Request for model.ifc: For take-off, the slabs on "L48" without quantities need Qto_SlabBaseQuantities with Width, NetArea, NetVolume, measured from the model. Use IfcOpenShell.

First a look at what the model holds.

```python
import ifcopenshell
import ifcopenshell.util.element
import ifcopenshell.util.unit

model = ifcopenshell.open("model.ifc")
print(model.schema)
for unit_type in ("LENGTHUNIT", "AREAUNIT", "VOLUMEUNIT"):
    print(unit_type, ifcopenshell.util.unit.calculate_unit_scale(model, unit_type))
storey = next(s for s in model.by_type("IfcBuildingStorey") if s.Name == "L48")
slabs = [e for e in ifcopenshell.util.element.get_decomposition(storey) if e.is_a("IfcSlab")]
for e in sorted(slabs, key=lambda e: e.id()):
    print(e.id(), e.is_a(), e.Name, list(ifcopenshell.util.element.get_psets(e, qtos_only=True)), sep=" | ")
```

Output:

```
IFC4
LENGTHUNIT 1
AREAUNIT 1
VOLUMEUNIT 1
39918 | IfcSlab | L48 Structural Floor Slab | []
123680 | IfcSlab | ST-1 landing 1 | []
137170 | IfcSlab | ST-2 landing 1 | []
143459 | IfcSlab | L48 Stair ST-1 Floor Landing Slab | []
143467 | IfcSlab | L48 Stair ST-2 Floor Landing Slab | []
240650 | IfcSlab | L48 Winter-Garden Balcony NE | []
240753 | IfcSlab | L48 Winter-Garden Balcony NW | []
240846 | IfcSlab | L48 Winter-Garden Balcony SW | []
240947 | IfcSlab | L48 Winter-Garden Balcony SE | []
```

```python
import ifcopenshell
import ifcopenshell.api.pset
import ifcopenshell.geom
import ifcopenshell.util.element
import ifcopenshell.util.shape
import ifcopenshell.util.unit

model = ifcopenshell.open("model.ifc")
unit_scale = ifcopenshell.util.unit.calculate_unit_scale(model)
area_scale = ifcopenshell.util.unit.calculate_unit_scale(model, "AREAUNIT")
volume_scale = ifcopenshell.util.unit.calculate_unit_scale(model, "VOLUMEUNIT")
settings = ifcopenshell.geom.settings()

storey = next(s for s in model.by_type("IfcBuildingStorey") if s.Name == "L48")
slabs = [e for e in ifcopenshell.util.element.get_decomposition(storey) if e.is_a("IfcSlab")]

for e in sorted(slabs, key=lambda e: e.id()):
    if ifcopenshell.util.element.get_psets(e, qtos_only=True, should_inherit=False):
        continue
    # Geometry comes back in metres, in the element's own axes.
    shape = ifcopenshell.geom.create_shape(settings, e)
    values = {
        "Width": ifcopenshell.util.shape.get_z(shape.geometry) / unit_scale,
        "NetArea": ifcopenshell.util.shape.get_footprint_area(shape.geometry) / area_scale,
        "NetVolume": ifcopenshell.util.shape.get_volume(shape.geometry) / volume_scale,
    }
    qto = ifcopenshell.api.pset.add_qto(model, product=e, name="Qto_SlabBaseQuantities")
    ifcopenshell.api.pset.edit_qto(model, qto=qto, properties=values)
    print(e.id(), {k: round(v, 3) for k, v in values.items()})

model.write("model_updated.ifc")
```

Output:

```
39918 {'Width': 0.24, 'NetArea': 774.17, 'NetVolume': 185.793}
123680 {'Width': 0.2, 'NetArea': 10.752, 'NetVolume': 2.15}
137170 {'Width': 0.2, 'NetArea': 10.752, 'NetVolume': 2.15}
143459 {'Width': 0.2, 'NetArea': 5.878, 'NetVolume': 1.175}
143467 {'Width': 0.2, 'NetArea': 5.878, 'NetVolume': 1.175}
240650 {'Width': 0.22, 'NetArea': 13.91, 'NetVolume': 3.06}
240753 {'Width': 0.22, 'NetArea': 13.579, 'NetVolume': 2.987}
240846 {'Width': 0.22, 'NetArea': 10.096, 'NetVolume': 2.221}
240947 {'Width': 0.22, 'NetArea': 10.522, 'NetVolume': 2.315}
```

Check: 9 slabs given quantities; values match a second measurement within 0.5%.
